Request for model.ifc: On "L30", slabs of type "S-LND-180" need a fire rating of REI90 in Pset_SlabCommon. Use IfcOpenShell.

First a look at what the model holds.

```python
import ifcopenshell
import ifcopenshell.util.element

model = ifcopenshell.open("model.ifc")
print(model.schema)
storey = next(s for s in model.by_type("IfcBuildingStorey") if s.Name == "L30")
slabs = [e for e in ifcopenshell.util.element.get_decomposition(storey) if e.is_a("IfcSlab")]
seen = {}
for e in slabs:
    element_type = ifcopenshell.util.element.get_type(e)
    key = (element_type.Name if element_type != e and element_type else None, ifcopenshell.util.element.get_pset(e, "Pset_SlabCommon", "FireRating"))
    seen[key] = seen.get(key, 0) + 1
for (name, value), count in sorted(seen.items(), key=str):
    print(count, "x", name, "|", value)
```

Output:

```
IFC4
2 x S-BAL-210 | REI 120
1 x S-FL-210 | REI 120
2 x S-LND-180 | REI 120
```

```python
import ifcopenshell
import ifcopenshell.api.pset
import ifcopenshell.util.element

model = ifcopenshell.open("model.ifc")

storey = next(s for s in model.by_type("IfcBuildingStorey") if s.Name == "L30")
slabs = [e for e in ifcopenshell.util.element.get_decomposition(storey) if e.is_a("IfcSlab")]

count = 0
for e in slabs:
    element_type = ifcopenshell.util.element.get_type(e)
    if element_type in (None, e) or element_type.Name != "S-LND-180":
        continue
    found = ifcopenshell.util.element.get_pset(e, "Pset_SlabCommon", should_inherit=False)
    if found:
        pset = model.by_id(found["id"])
        if len(ifcopenshell.util.element.get_elements_by_pset(pset)) > 1:
            pset = ifcopenshell.api.pset.unshare_pset(model, products=[e], pset=pset)[0]
    else:
        pset = ifcopenshell.api.pset.add_pset(model, product=e, name="Pset_SlabCommon")
    ifcopenshell.api.pset.edit_pset(model, pset=pset, properties={"FireRating": "REI90"})
    count += 1

print(count, "slabs updated")

model.write("model_rev.ifc")
```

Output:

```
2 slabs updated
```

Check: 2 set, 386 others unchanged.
